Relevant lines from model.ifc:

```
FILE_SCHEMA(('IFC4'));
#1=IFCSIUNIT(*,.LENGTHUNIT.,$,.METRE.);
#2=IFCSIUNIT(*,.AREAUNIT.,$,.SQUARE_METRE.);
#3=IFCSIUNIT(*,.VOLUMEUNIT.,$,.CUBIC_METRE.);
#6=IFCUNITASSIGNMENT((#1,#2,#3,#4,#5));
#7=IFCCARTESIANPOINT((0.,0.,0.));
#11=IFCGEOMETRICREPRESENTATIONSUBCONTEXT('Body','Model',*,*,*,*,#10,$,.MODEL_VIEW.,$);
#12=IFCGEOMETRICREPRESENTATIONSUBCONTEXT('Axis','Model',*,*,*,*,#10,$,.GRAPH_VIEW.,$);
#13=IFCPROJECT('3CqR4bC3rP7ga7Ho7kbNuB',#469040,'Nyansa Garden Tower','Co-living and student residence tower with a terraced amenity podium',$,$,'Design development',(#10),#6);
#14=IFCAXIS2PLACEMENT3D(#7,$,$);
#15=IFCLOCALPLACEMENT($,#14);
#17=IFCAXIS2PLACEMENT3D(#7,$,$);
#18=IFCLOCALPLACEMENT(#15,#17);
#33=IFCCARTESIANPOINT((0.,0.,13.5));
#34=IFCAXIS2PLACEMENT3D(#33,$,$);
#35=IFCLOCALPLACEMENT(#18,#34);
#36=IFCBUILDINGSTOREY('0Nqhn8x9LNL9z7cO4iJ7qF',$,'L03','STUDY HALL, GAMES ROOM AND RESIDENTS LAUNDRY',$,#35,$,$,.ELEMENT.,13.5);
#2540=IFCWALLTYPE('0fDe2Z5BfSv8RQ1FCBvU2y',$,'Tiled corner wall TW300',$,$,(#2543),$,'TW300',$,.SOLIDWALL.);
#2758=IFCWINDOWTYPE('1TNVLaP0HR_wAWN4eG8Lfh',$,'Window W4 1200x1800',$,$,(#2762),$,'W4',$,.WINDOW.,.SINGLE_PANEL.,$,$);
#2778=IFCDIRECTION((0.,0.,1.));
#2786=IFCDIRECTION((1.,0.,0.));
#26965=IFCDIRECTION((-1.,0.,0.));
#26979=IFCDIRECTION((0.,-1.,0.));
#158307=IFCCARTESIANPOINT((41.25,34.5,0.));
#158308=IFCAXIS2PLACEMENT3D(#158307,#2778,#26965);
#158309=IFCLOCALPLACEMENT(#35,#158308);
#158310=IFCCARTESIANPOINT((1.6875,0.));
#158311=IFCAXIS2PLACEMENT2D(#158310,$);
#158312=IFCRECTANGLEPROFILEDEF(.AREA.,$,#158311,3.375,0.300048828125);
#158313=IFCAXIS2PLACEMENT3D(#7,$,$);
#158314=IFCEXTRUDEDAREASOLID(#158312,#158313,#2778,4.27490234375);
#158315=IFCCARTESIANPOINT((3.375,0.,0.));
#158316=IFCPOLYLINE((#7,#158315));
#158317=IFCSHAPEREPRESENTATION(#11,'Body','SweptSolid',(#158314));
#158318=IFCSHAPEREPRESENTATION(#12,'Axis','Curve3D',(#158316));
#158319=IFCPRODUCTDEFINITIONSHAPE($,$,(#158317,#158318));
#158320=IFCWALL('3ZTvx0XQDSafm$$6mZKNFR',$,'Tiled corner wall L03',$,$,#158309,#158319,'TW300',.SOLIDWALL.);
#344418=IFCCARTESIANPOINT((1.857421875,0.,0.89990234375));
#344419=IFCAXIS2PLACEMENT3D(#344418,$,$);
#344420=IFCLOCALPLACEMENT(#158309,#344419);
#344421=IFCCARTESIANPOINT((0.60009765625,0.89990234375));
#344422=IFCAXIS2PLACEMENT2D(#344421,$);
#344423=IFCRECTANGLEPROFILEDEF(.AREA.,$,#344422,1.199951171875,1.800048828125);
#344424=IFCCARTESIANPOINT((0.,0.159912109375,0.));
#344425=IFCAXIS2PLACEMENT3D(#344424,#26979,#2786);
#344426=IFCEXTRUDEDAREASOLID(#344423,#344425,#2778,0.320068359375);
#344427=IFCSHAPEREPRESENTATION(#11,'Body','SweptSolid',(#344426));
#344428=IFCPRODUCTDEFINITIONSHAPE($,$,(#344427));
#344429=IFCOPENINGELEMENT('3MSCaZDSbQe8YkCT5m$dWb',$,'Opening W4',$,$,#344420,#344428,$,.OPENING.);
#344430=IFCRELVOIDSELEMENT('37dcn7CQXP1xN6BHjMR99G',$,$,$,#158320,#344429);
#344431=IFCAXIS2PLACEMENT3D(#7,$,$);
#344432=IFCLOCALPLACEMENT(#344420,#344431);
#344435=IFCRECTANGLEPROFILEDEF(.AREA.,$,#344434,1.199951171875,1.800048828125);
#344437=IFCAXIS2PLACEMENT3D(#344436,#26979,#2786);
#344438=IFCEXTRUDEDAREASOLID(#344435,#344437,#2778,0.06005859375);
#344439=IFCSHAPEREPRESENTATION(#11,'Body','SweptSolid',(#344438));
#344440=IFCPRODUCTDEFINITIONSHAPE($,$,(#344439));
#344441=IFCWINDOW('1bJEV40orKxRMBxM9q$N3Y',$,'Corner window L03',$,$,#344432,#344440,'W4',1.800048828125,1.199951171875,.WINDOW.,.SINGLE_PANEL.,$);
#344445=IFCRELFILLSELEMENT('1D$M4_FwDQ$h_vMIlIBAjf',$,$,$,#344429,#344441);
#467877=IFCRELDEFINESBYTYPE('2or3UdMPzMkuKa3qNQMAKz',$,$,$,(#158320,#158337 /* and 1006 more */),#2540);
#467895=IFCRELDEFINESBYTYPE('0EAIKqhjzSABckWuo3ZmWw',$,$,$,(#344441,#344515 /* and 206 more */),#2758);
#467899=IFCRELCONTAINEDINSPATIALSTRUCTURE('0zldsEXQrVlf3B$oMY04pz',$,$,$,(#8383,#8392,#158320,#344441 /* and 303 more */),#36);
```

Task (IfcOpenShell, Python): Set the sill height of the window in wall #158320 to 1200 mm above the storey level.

```python
import numpy as np
import ifcopenshell
import ifcopenshell.api.geometry
import ifcopenshell.geom
import ifcopenshell.util.element
import ifcopenshell.util.placement
import ifcopenshell.util.shape
import ifcopenshell.util.unit

model = ifcopenshell.open("model.ifc")
unit_scale = ifcopenshell.util.unit.calculate_unit_scale(model)

window = model.by_id(344441)
opening = window.FillsVoids[0].RelatingOpeningElement
storey = ifcopenshell.util.element.get_container(window, ifc_class="IfcBuildingStorey")
level = ifcopenshell.util.placement.get_local_placement(storey.ObjectPlacement)[2, 3]

# The opening's origin need not be at the sill, so measure its lowest point.
shape = ifcopenshell.geom.create_shape(ifcopenshell.geom.settings(), opening)
bottom = ifcopenshell.util.shape.get_shape_bottom_elevation(shape, shape.geometry) / unit_scale
dz = level + 1.2 / unit_scale - bottom

shift = np.array([0.0, 0.0, dz])
# The window is placed relative to its opening, so it follows when the opening moves.
matrix = ifcopenshell.util.placement.get_local_placement(opening.ObjectPlacement)
matrix[:3, 3] += shift
ifcopenshell.api.geometry.edit_object_placement(
    model, product=opening, matrix=matrix, is_si=False, should_transform_children=True
)

print(f"moved by {dz * unit_scale:+.3f} m")

model.write("model_rev.ifc")
```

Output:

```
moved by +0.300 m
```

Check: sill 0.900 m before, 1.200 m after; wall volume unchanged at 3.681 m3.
